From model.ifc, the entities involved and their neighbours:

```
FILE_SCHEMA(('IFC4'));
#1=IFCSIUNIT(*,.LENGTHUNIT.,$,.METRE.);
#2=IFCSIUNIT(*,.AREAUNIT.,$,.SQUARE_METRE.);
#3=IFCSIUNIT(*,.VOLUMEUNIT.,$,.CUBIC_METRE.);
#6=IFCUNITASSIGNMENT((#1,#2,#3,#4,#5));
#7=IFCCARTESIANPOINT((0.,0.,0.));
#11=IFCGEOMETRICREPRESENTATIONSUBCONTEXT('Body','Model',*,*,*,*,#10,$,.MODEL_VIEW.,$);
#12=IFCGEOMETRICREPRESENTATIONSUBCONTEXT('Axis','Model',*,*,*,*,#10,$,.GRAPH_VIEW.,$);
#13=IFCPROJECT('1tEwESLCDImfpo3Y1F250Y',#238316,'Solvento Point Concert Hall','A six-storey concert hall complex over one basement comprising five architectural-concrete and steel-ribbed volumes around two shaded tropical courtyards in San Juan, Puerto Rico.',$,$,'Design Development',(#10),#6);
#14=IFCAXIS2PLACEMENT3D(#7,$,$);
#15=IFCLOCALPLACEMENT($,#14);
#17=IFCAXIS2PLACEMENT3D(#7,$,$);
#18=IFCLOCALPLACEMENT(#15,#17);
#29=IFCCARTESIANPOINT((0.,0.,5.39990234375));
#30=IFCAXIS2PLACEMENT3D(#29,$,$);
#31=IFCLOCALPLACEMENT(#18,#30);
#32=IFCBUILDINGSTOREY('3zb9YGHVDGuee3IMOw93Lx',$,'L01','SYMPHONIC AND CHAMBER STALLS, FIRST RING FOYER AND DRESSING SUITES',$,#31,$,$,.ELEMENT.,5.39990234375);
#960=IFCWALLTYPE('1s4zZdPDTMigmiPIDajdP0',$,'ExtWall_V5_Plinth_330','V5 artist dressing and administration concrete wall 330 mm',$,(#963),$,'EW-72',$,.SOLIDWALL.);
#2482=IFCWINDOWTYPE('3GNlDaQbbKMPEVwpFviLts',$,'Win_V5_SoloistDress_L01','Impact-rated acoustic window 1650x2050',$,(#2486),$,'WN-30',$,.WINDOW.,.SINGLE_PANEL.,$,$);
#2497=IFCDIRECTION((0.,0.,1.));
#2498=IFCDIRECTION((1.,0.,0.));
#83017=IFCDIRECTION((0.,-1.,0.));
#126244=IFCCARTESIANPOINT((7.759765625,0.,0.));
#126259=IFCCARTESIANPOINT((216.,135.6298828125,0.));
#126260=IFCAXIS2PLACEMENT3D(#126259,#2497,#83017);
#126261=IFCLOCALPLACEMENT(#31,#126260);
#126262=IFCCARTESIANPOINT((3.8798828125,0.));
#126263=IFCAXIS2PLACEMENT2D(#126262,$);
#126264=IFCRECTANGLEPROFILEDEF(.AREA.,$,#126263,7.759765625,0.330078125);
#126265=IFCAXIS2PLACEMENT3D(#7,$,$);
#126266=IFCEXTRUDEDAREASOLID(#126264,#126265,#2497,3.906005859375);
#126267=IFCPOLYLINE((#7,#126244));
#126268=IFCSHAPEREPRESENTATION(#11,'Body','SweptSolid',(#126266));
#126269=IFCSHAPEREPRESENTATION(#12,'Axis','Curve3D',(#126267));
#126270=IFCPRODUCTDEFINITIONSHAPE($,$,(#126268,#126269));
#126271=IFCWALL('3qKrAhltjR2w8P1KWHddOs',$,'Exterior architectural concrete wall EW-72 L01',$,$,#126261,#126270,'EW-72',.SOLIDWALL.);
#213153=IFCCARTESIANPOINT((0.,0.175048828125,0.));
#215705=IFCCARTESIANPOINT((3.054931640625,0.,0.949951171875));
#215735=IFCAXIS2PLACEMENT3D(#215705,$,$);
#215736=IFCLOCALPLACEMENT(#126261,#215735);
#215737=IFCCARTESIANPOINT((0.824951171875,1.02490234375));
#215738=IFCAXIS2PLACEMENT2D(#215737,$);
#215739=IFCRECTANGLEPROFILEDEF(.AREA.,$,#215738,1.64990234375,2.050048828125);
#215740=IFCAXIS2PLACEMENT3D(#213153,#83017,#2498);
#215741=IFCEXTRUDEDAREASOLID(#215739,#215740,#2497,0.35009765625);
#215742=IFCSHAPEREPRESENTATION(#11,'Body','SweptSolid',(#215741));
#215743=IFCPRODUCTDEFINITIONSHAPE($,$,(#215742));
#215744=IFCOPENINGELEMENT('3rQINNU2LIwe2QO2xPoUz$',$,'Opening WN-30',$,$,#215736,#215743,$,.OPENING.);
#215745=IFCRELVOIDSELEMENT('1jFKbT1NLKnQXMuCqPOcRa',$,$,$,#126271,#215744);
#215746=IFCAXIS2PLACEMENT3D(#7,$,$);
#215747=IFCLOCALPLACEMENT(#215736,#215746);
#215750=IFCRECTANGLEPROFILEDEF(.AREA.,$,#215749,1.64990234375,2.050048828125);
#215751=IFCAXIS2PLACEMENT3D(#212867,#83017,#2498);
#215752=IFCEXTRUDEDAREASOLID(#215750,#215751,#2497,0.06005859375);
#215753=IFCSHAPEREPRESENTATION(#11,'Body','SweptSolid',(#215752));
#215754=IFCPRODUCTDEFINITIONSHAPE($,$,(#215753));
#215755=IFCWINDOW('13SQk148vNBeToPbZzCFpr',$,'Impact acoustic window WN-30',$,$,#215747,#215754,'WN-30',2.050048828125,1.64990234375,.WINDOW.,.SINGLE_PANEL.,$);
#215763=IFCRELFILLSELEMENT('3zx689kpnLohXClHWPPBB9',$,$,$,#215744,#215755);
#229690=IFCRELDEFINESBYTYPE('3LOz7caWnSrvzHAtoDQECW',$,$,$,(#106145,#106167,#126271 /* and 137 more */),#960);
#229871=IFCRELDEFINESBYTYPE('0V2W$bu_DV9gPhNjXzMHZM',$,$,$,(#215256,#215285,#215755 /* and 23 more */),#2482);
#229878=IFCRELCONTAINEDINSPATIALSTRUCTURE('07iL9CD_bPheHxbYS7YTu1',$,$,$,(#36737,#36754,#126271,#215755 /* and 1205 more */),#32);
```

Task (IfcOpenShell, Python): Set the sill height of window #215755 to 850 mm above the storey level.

```python
import numpy as np
import ifcopenshell
import ifcopenshell.api.geometry
import ifcopenshell.geom
import ifcopenshell.util.element
import ifcopenshell.util.placement
import ifcopenshell.util.shape
import ifcopenshell.util.unit

model = ifcopenshell.open("model.ifc")
unit_scale = ifcopenshell.util.unit.calculate_unit_scale(model)

window = model.by_id(215755)
opening = window.FillsVoids[0].RelatingOpeningElement
storey = ifcopenshell.util.element.get_container(window, ifc_class="IfcBuildingStorey")
level = ifcopenshell.util.placement.get_local_placement(storey.ObjectPlacement)[2, 3]

# The opening's origin need not be at the sill, so measure its lowest point.
shape = ifcopenshell.geom.create_shape(ifcopenshell.geom.settings(), opening)
bottom = ifcopenshell.util.shape.get_shape_bottom_elevation(shape, shape.geometry) / unit_scale
dz = level + 0.85 - bottom

shift = np.array([0.0, 0.0, dz])
# The window is placed relative to its opening, so it follows when the opening moves.
matrix = ifcopenshell.util.placement.get_local_placement(opening.ObjectPlacement)
matrix[:3, 3] += shift
ifcopenshell.api.geometry.edit_object_placement(
    model, product=opening, matrix=matrix, is_si=False, should_transform_children=True
)

print(f"moved by {dz * unit_scale:+.3f} m")

model.write("model_rev.ifc")
```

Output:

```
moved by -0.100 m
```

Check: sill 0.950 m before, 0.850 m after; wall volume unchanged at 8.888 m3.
